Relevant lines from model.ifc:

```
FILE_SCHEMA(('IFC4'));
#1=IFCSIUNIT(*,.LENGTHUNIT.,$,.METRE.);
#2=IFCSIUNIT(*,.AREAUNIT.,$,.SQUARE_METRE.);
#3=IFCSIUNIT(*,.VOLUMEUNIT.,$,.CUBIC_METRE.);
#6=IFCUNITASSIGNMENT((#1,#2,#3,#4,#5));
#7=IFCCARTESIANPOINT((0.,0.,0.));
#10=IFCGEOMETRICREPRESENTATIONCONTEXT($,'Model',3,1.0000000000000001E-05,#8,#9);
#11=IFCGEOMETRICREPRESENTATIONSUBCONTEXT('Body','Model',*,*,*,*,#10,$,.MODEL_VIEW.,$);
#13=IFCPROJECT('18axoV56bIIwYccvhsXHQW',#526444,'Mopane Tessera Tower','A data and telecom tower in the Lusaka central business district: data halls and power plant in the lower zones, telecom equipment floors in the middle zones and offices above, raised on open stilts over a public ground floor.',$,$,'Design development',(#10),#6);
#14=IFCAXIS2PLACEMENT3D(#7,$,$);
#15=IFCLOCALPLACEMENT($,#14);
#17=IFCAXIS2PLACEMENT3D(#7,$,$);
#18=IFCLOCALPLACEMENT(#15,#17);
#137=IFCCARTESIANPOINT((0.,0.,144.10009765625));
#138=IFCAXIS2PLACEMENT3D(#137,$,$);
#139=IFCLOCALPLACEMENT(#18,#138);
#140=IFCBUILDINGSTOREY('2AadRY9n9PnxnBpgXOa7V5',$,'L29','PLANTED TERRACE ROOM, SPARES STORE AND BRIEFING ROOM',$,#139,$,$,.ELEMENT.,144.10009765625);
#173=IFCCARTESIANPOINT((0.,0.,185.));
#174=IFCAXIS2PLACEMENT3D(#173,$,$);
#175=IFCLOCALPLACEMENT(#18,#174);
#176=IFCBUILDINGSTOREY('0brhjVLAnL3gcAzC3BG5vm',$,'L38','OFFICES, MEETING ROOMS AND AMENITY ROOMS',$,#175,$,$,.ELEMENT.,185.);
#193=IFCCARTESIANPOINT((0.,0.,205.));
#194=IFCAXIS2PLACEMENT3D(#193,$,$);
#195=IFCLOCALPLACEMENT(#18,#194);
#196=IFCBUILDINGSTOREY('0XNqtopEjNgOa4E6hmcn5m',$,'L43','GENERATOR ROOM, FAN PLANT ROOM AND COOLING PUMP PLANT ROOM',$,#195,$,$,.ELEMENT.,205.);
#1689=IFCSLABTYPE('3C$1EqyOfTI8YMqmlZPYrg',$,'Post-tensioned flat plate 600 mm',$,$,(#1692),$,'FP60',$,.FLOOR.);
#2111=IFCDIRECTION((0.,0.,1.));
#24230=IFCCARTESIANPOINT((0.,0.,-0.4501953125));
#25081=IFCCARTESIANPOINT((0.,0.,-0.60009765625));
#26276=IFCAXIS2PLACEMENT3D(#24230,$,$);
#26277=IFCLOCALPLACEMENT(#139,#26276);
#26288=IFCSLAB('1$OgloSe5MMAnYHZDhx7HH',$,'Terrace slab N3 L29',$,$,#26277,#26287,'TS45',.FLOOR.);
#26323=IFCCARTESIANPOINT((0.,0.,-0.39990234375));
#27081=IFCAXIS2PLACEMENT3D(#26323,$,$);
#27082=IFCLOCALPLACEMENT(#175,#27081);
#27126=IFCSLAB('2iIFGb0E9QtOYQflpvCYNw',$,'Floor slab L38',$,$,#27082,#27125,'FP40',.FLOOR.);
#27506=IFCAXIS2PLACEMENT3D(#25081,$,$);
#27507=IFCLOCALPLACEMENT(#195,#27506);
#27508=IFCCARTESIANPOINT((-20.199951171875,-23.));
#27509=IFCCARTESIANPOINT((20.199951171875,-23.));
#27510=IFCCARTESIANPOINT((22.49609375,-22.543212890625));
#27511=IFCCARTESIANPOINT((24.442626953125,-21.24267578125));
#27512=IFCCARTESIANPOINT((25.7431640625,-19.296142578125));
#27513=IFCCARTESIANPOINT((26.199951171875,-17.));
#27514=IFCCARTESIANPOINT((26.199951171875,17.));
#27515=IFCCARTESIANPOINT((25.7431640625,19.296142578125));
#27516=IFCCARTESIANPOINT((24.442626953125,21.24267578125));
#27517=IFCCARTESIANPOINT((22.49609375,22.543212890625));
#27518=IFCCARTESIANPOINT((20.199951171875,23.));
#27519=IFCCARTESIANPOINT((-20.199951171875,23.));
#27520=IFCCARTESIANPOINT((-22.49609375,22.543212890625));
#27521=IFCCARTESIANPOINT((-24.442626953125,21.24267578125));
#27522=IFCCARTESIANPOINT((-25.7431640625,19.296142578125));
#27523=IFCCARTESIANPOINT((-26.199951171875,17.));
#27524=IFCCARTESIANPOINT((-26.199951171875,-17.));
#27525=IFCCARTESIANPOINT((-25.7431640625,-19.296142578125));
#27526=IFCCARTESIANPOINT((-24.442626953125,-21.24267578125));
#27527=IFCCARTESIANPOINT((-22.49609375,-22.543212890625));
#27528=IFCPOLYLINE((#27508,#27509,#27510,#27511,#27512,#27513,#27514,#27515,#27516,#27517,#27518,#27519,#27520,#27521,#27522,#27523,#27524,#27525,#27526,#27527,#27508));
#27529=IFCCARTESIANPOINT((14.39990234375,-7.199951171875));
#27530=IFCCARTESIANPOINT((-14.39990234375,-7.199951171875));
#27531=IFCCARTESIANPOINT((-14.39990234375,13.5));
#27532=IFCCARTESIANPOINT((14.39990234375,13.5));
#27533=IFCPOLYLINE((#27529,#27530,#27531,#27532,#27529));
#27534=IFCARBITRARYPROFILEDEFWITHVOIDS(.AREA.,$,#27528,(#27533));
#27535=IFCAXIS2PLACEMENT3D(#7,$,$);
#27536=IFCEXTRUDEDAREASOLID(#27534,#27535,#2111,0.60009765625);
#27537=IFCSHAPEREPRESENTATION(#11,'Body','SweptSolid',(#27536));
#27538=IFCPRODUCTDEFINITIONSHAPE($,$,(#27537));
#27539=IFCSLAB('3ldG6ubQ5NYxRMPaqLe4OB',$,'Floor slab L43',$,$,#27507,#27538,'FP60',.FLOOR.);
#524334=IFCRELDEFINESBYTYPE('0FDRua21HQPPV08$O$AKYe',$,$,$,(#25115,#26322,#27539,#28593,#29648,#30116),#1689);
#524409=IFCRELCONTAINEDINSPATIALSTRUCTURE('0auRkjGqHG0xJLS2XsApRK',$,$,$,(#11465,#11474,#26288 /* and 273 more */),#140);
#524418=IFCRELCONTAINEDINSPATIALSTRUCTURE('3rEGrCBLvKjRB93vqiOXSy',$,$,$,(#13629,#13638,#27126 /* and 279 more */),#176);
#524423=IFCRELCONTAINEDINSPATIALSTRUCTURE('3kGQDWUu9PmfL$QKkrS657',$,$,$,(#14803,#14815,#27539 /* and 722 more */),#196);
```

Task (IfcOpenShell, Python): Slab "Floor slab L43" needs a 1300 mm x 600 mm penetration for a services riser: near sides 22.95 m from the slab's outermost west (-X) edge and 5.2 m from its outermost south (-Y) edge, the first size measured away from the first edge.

```python
import numpy as np
import ifcopenshell
import ifcopenshell.api.feature
import ifcopenshell.api.geometry
import ifcopenshell.api.root
import ifcopenshell.geom
import ifcopenshell.util.placement
import ifcopenshell.util.representation
import ifcopenshell.util.shape
import ifcopenshell.util.unit

model = ifcopenshell.open("model.ifc")
unit_scale = ifcopenshell.util.unit.calculate_unit_scale(model)
settings = ifcopenshell.geom.settings()


def volume(element):
    """Net volume in cubic metres, openings subtracted."""
    shape = ifcopenshell.geom.create_shape(settings, element)
    return ifcopenshell.util.shape.get_volume(shape.geometry)


slab = model.by_guid("3ldG6ubQ5NYxRMPaqLe4OB")
before = volume(slab)

# Extent in the slab's own axes, in metres. The edges named are its -X and -Y sides.
slab_shape = ifcopenshell.geom.create_shape(settings, slab)
vertices = ifcopenshell.util.shape.get_vertices(slab_shape.geometry)
x_min, y_min, bottom = vertices.min(axis=0)
top = vertices[:, 2].max()

opening = ifcopenshell.api.root.create_entity(model, ifc_class="IfcOpeningElement", name="Services riser opening", predefined_type="OPENING")
context = ifcopenshell.util.representation.get_context(model, "Model", "Body", "MODEL_VIEW")
width, depth = 1.3, 0.6
outline = [(0.0, 0.0), (width, 0.0), (width, depth), (0.0, depth), (0.0, 0.0)]
# Overshoot both faces by 50 mm so the cut is clean.
shape = ifcopenshell.api.geometry.add_slab_representation(
    model, context=context, depth=top - bottom + 0.1, polyline=outline
)
ifcopenshell.api.geometry.assign_representation(model, product=opening, representation=shape)

matrix = ifcopenshell.util.placement.get_local_placement(slab.ObjectPlacement)
matrix[:, 3] = matrix @ np.append(np.array([x_min + 22.95, y_min + 5.2, bottom - 0.05]) / unit_scale, 1.0)
ifcopenshell.api.geometry.edit_object_placement(model, product=opening, matrix=matrix, is_si=False)
ifcopenshell.api.feature.add_feature(model, feature=opening, element=slab)

after = volume(slab)

print(f"slab volume {before:.3f} -> {after:.3f} m3")

model.write("model-out.ifc")
```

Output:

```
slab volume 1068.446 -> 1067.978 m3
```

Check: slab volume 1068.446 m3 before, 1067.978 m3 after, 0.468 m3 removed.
